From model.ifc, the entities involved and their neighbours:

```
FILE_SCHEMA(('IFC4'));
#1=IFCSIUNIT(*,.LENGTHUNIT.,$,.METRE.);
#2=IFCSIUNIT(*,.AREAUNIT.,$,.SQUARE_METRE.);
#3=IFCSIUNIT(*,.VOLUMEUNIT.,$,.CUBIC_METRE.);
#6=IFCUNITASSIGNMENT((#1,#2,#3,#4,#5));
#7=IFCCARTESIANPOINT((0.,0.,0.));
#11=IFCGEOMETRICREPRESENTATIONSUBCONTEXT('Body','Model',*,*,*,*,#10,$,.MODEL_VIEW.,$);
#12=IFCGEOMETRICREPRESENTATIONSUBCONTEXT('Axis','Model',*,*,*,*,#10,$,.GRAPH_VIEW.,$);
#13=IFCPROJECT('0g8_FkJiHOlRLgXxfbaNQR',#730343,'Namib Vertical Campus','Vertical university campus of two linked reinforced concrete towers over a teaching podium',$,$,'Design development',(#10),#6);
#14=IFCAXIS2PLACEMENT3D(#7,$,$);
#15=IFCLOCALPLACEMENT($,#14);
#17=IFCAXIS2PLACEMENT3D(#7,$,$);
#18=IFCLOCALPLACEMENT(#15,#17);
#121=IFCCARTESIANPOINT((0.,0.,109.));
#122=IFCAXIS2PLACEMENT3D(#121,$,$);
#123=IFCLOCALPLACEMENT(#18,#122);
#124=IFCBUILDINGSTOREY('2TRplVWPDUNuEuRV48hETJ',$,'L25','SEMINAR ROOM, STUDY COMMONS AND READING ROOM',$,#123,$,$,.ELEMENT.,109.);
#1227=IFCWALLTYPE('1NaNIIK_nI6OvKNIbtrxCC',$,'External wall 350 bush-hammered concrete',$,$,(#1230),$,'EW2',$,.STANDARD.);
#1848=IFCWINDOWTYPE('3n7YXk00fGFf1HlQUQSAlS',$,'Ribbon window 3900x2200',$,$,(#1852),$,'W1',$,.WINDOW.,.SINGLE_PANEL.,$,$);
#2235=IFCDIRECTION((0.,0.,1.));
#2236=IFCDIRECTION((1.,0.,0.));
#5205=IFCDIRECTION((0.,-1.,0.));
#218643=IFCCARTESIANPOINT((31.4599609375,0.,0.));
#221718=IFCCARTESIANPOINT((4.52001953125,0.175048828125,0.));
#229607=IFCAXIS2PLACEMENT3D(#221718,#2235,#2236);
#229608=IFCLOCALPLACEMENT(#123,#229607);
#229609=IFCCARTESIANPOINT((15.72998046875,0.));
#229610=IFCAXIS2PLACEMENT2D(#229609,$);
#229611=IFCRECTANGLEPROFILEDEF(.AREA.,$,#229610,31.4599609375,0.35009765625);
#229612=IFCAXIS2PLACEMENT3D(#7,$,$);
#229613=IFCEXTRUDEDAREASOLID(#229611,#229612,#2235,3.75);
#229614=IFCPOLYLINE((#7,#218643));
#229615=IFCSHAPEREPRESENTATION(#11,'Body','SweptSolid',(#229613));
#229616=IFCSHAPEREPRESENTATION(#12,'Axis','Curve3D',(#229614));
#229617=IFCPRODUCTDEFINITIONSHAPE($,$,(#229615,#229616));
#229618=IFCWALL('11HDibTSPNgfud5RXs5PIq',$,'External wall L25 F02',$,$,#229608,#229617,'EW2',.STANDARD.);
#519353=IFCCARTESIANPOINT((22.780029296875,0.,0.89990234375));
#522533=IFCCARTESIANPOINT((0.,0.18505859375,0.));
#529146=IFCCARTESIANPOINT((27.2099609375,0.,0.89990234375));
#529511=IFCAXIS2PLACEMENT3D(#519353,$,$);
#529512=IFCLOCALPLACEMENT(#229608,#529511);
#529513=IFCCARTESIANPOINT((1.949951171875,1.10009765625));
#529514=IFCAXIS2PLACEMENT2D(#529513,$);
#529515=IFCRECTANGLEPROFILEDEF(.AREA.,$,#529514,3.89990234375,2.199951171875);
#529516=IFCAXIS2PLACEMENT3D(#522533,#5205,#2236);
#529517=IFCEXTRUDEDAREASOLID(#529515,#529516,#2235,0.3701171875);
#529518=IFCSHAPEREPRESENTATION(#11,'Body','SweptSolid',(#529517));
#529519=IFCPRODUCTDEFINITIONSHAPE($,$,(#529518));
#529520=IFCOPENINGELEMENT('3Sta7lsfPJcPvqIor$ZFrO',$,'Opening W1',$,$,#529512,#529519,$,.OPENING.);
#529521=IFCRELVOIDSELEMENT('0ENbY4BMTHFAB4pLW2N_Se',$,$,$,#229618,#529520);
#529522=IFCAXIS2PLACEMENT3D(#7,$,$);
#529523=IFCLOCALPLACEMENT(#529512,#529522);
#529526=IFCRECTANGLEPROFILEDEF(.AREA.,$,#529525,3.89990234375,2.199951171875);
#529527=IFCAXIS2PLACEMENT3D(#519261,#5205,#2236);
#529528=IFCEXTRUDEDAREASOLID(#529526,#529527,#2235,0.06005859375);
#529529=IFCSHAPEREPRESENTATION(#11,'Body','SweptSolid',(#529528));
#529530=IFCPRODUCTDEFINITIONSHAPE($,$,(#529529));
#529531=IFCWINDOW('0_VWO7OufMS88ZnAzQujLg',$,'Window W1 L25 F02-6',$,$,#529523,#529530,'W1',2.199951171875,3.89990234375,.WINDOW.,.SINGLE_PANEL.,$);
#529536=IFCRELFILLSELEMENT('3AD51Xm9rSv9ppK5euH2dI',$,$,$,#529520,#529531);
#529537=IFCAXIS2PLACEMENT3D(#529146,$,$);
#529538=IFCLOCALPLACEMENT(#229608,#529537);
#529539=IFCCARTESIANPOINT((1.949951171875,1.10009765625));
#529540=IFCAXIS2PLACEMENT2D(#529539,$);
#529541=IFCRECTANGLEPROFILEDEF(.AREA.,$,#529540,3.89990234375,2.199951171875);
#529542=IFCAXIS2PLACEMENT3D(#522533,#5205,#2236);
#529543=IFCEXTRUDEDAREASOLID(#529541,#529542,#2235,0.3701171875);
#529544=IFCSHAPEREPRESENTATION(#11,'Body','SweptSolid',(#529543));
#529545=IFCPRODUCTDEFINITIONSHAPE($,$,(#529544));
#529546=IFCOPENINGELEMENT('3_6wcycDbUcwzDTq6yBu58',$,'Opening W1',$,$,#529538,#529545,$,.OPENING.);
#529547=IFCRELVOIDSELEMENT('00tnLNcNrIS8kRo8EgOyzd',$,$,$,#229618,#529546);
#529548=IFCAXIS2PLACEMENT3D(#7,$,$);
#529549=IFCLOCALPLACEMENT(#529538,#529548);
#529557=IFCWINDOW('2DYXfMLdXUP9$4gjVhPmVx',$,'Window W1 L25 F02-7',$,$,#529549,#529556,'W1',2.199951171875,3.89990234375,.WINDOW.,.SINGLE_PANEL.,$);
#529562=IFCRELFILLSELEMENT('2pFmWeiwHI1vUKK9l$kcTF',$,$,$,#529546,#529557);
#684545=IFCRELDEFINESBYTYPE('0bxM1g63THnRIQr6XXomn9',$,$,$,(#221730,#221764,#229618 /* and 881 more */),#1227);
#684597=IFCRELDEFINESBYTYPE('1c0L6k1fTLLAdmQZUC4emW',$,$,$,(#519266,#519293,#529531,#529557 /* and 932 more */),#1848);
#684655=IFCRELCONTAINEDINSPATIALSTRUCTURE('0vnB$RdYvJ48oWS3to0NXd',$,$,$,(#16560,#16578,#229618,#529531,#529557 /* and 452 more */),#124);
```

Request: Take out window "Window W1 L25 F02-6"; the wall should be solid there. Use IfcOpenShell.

```python
import ifcopenshell
import ifcopenshell.api.feature
import ifcopenshell.api.root
import ifcopenshell.geom
import ifcopenshell.util.shape

model = ifcopenshell.open("model.ifc")
settings = ifcopenshell.geom.settings()


def volume(element):
    """Net volume in cubic metres, openings subtracted."""
    shape = ifcopenshell.geom.create_shape(settings, element)
    return ifcopenshell.util.shape.get_volume(shape.geometry)


window = model.by_guid("0_VWO7OufMS88ZnAzQujLg")
opening = window.FillsVoids[0].RelatingOpeningElement
wall = opening.VoidsElements[0].RelatingBuildingElement
before = volume(wall)

ifcopenshell.api.root.remove_product(model, product=window)
ifcopenshell.api.feature.remove_feature(model, feature=opening)

after = volume(wall)

print(f"wall volume {before:.3f} -> {after:.3f} m3")

model.write("model_edited.ifc")
```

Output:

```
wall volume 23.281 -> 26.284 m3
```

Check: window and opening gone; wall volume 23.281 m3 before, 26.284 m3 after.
